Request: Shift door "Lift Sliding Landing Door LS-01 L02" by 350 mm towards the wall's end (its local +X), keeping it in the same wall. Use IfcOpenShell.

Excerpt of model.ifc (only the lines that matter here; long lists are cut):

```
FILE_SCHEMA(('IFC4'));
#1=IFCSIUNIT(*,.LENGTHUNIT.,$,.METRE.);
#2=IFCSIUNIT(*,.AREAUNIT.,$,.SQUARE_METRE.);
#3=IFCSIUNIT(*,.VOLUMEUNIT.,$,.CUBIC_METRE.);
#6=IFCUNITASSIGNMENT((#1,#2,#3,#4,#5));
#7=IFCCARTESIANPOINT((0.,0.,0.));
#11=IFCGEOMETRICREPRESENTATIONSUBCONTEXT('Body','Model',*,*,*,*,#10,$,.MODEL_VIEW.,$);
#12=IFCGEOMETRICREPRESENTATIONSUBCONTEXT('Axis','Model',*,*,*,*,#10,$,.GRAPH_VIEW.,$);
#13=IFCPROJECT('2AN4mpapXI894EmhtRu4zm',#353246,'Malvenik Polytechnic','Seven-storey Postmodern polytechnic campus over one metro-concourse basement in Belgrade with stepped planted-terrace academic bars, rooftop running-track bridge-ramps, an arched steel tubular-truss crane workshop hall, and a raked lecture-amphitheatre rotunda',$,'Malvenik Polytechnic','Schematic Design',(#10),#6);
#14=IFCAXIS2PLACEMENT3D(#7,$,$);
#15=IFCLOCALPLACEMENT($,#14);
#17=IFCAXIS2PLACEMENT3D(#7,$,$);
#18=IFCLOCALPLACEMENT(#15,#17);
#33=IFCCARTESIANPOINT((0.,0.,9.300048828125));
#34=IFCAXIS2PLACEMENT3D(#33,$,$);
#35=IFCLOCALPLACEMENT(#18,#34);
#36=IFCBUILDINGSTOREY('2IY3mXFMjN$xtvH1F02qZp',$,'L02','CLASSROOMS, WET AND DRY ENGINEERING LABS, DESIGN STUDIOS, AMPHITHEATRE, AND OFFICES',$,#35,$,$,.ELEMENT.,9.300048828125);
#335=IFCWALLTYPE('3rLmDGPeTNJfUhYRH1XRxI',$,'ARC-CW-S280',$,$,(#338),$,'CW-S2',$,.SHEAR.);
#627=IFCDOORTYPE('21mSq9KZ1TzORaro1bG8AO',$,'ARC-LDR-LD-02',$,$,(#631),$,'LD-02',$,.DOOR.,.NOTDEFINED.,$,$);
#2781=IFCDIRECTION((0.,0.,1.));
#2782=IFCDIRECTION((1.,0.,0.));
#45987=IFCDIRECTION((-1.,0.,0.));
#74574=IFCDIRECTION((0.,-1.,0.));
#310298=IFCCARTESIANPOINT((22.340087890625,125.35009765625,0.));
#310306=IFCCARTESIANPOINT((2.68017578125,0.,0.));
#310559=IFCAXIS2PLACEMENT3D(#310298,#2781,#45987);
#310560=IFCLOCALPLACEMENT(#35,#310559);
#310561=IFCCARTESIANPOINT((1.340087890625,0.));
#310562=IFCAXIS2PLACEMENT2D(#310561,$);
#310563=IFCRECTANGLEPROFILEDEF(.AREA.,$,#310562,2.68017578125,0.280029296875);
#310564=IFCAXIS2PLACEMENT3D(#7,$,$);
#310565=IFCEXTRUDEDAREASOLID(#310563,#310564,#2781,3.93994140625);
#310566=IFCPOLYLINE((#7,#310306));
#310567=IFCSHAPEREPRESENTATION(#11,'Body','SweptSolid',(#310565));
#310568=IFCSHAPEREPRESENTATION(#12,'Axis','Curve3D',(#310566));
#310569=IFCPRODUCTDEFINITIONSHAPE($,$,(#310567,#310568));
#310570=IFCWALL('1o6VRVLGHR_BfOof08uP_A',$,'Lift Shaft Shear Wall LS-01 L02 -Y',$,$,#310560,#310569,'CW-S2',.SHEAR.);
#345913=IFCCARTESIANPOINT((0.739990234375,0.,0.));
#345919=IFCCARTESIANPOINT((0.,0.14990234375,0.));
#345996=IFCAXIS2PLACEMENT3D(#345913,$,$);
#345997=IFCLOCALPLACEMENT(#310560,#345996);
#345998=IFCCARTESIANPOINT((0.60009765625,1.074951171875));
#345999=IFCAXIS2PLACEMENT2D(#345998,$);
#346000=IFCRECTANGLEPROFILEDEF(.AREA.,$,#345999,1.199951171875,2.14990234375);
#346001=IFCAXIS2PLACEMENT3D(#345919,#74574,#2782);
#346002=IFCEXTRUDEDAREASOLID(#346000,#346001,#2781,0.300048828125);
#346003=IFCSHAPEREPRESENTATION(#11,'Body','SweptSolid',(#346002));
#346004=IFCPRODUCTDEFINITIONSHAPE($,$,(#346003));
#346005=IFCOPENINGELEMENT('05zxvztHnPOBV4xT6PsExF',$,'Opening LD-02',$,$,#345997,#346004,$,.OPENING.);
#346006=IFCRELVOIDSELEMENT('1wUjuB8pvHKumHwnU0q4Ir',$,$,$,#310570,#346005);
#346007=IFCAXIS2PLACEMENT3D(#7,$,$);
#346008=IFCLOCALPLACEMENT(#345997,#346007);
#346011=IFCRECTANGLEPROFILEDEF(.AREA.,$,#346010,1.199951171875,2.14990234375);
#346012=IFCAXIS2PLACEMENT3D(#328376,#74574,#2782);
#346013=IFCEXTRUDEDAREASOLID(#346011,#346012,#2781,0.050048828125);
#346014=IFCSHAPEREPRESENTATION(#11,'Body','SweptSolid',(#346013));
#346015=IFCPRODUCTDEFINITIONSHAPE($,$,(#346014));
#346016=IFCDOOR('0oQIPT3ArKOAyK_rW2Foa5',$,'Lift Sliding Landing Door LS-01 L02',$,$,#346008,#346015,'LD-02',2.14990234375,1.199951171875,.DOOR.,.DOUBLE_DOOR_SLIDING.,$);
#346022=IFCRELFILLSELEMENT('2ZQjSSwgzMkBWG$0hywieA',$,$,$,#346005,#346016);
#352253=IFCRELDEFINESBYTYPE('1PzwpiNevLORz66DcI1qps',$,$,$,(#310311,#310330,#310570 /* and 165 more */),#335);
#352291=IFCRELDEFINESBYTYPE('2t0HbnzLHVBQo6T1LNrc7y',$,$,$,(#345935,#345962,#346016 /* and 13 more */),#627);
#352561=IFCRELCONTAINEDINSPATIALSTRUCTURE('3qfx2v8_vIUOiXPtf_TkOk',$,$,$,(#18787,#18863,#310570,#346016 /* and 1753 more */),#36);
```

```python
import ifcopenshell
import ifcopenshell.api.geometry
import ifcopenshell.util.placement
import ifcopenshell.util.unit

model = ifcopenshell.open("model.ifc")
unit_scale = ifcopenshell.util.unit.calculate_unit_scale(model)

door = model.by_guid("0oQIPT3ArKOAyK_rW2Foa5")
opening = door.FillsVoids[0].RelatingOpeningElement
wall = opening.VoidsElements[0].RelatingBuildingElement

wall_matrix = ifcopenshell.util.placement.get_local_placement(wall.ObjectPlacement)
shift = wall_matrix[:3, 0] * 0.35 / unit_scale
before = ifcopenshell.util.placement.get_local_placement(door.ObjectPlacement)[:3, 3].copy()

# The door is placed relative to its opening, so it follows when the opening moves.
matrix = ifcopenshell.util.placement.get_local_placement(opening.ObjectPlacement)
matrix[:3, 3] += shift
ifcopenshell.api.geometry.edit_object_placement(
    model, product=opening, matrix=matrix, is_si=False, should_transform_children=True
)

after = ifcopenshell.util.placement.get_local_placement(door.ObjectPlacement)[:3, 3]
print("door moved by", (after - before).round(3) + 0.0)

model.write("model_v2.ifc")
```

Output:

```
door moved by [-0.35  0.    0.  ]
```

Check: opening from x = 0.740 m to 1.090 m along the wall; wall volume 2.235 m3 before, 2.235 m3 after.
